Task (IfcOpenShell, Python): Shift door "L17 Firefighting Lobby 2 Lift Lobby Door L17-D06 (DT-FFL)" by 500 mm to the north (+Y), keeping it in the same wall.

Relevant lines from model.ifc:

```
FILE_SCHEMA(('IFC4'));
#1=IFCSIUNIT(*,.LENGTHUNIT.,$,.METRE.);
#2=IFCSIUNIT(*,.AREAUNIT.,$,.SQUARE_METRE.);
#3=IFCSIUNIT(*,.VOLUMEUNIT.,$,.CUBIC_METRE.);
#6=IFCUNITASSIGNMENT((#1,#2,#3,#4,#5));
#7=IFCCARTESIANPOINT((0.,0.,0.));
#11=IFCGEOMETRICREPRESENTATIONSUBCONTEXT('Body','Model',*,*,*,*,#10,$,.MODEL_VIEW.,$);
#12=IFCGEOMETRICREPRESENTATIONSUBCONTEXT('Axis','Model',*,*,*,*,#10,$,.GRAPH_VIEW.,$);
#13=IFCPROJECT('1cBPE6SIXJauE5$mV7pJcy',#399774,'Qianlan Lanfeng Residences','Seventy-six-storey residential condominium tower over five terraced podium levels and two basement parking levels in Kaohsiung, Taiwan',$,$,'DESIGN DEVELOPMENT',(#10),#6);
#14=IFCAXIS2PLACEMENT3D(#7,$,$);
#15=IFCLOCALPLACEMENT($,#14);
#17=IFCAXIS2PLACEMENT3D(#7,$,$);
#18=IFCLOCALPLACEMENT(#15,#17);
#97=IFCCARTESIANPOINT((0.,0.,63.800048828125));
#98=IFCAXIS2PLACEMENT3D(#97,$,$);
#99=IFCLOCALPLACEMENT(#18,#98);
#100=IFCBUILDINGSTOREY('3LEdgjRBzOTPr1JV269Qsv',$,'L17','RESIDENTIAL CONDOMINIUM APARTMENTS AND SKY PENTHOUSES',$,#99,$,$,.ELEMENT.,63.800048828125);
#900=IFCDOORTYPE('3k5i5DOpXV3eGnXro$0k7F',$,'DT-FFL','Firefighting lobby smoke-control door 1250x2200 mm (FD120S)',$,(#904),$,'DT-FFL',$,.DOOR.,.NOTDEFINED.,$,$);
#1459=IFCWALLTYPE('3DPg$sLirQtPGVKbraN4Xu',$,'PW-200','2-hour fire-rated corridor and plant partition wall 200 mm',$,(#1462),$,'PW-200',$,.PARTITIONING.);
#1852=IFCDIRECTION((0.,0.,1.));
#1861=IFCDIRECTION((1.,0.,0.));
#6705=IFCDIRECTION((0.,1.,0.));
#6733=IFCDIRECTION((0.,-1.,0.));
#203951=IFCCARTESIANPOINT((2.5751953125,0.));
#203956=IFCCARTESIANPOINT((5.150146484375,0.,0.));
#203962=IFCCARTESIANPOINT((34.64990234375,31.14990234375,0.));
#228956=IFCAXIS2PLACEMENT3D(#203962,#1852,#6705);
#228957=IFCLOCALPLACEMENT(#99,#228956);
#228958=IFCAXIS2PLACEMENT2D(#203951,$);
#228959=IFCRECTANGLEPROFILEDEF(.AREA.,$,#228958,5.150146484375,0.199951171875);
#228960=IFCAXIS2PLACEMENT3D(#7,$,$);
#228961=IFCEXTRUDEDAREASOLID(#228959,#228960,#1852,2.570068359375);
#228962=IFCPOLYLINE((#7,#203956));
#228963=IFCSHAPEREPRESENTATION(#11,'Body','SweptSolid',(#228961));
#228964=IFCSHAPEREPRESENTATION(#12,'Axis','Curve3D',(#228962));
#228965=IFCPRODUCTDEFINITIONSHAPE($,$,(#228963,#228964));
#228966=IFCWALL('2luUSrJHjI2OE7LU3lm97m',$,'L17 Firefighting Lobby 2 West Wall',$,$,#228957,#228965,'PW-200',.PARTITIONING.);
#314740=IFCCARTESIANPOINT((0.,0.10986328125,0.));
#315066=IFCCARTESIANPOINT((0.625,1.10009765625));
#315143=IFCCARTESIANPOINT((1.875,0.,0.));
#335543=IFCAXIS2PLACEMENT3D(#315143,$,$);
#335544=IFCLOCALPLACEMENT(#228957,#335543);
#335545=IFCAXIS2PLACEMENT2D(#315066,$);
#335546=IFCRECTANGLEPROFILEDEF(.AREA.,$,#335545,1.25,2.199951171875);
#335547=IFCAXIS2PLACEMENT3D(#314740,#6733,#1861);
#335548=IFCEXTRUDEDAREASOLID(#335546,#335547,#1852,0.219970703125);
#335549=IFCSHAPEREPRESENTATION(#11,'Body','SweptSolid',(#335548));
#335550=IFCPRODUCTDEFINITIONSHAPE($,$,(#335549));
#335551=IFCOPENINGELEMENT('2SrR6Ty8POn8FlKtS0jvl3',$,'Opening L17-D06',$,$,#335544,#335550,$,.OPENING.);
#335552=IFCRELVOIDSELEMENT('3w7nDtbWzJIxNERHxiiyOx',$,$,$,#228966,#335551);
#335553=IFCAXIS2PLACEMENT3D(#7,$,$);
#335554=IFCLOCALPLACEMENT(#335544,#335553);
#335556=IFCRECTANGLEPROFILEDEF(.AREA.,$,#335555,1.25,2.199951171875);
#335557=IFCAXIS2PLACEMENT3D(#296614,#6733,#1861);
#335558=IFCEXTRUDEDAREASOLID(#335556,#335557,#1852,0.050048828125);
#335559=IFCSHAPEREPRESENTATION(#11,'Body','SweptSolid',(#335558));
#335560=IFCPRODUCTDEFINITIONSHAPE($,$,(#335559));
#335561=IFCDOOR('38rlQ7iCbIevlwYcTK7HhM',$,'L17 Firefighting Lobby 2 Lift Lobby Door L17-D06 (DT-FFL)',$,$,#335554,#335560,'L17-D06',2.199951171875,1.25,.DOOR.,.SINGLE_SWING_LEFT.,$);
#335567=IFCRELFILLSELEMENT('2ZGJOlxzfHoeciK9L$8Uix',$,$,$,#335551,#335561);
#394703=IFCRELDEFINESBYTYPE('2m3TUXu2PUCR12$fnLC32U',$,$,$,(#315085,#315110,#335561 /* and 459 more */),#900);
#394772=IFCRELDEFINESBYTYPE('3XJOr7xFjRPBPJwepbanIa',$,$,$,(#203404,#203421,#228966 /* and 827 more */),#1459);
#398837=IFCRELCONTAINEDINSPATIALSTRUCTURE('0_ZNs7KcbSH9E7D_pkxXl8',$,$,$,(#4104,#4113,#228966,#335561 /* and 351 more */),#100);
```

```python
import ifcopenshell
import ifcopenshell.api.geometry
import ifcopenshell.util.placement

model = ifcopenshell.open("model.ifc")

door = model.by_guid("38rlQ7iCbIevlwYcTK7HhM")
opening = door.FillsVoids[0].RelatingOpeningElement
wall = opening.VoidsElements[0].RelatingBuildingElement

wall_matrix = ifcopenshell.util.placement.get_local_placement(wall.ObjectPlacement)
shift = wall_matrix[:3, 0] * 0.5
before = ifcopenshell.util.placement.get_local_placement(door.ObjectPlacement)[:3, 3].copy()

# The door is placed relative to its opening, so it follows when the opening moves.
matrix = ifcopenshell.util.placement.get_local_placement(opening.ObjectPlacement)
matrix[:3, 3] += shift
ifcopenshell.api.geometry.edit_object_placement(
    model, product=opening, matrix=matrix, is_si=False, should_transform_children=True
)

after = ifcopenshell.util.placement.get_local_placement(door.ObjectPlacement)[:3, 3]
print("door moved by", (after - before).round(3) + 0.0)

model.write("model_updated.ifc")
```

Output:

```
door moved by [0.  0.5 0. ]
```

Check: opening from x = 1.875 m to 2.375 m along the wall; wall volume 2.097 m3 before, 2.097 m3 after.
